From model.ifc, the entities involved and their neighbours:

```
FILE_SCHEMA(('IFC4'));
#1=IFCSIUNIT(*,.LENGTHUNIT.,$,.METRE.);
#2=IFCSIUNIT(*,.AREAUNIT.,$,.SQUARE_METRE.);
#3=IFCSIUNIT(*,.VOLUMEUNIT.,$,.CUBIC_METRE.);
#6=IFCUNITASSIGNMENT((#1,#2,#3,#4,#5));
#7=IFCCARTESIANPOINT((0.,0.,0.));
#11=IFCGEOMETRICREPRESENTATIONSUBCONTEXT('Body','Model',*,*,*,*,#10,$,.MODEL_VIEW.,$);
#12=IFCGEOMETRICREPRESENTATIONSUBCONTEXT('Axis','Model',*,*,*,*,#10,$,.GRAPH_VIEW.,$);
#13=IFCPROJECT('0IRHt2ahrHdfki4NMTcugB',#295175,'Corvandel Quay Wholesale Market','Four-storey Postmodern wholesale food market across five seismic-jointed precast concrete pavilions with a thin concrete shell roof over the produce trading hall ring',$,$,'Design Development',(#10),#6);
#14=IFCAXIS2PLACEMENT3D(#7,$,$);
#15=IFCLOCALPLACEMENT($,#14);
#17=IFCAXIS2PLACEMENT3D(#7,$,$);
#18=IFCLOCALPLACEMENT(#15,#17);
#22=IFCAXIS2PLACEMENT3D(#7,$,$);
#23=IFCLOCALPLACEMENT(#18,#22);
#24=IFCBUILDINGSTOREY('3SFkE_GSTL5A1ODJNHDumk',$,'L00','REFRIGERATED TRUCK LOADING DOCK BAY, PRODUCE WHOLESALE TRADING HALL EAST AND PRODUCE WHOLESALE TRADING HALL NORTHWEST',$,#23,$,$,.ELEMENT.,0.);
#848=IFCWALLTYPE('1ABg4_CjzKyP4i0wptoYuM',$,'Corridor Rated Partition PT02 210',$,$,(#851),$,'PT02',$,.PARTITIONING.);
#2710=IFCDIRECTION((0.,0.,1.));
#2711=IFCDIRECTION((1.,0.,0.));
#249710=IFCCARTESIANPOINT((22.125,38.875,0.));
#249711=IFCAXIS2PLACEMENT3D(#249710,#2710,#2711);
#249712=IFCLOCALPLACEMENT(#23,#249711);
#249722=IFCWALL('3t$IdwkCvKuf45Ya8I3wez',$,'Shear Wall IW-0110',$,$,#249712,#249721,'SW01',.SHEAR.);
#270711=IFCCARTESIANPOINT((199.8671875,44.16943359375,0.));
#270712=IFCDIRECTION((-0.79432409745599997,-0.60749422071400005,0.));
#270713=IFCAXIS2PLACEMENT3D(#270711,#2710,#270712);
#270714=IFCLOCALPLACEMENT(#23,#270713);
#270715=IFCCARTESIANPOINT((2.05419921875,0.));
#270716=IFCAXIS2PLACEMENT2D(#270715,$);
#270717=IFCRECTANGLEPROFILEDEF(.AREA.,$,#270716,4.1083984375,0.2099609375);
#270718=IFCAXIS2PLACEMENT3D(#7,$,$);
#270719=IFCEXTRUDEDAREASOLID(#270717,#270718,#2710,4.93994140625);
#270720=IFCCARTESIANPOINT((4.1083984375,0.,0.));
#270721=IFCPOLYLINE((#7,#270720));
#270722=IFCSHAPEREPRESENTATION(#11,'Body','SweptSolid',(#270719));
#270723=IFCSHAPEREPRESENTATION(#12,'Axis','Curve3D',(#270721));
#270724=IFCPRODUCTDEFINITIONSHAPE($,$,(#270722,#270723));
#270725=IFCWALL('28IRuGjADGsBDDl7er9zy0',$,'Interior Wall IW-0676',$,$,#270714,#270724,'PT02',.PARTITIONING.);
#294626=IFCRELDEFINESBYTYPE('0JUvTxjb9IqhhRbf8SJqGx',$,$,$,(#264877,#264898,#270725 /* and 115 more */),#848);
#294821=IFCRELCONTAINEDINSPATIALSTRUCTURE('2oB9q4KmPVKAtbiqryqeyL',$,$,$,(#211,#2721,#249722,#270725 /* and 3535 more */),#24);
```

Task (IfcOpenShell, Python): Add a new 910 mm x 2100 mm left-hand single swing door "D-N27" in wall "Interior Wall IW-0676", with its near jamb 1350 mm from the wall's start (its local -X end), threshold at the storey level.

```python
import numpy as np
import ifcopenshell
import ifcopenshell.api.feature
import ifcopenshell.api.geometry
import ifcopenshell.api.root
import ifcopenshell.api.spatial
import ifcopenshell.geom
import ifcopenshell.util.element
import ifcopenshell.util.placement
import ifcopenshell.util.representation
import ifcopenshell.util.shape
import ifcopenshell.util.unit

model = ifcopenshell.open("model.ifc")
unit_scale = ifcopenshell.util.unit.calculate_unit_scale(model)
settings = ifcopenshell.geom.settings()


def volume(element):
    """Net volume in cubic metres, openings subtracted."""
    shape = ifcopenshell.geom.create_shape(settings, element)
    return ifcopenshell.util.shape.get_volume(shape.geometry)


wall = model.by_guid("28IRuGjADGsBDDl7er9zy0")
storey = ifcopenshell.util.element.get_container(wall, ifc_class="IfcBuildingStorey")
context = ifcopenshell.util.representation.get_context(model, "Model", "Body", "MODEL_VIEW")
before = volume(wall)

width, height, from_end, sill = 0.91, 2.1, 1.35, 0.0  # metres

# The wall runs along its own X axis, and the end named is its -X end.
wall_shape = ifcopenshell.geom.create_shape(settings, wall)
x, y, z = ifcopenshell.util.shape.get_vertices(wall_shape.geometry).T
start = x.min() + from_end
face, thickness = float(y.min()), float(y.max() - y.min())
wall_matrix = ifcopenshell.util.placement.get_local_placement(wall.ObjectPlacement)
level = ifcopenshell.util.placement.get_local_placement(storey.ObjectPlacement)[2, 3]


def in_wall(x, y):
    """Placement at x, y metres in the wall's axes, at sill height."""
    matrix = wall_matrix.copy()
    matrix[:, 3] = wall_matrix @ np.array([x / unit_scale, y / unit_scale, 0.0, 1.0])
    matrix[2, 3] = level + sill / unit_scale
    return matrix


# Opening: a box that overshoots both wall faces by 50 mm.
opening = ifcopenshell.api.root.create_entity(model, ifc_class="IfcOpeningElement", predefined_type="OPENING")
box = ifcopenshell.api.geometry.add_wall_representation(
    model, context=context, length=width, height=height, thickness=thickness + 0.1
)
ifcopenshell.api.geometry.assign_representation(model, product=opening, representation=box)
ifcopenshell.api.geometry.edit_object_placement(model, product=opening, matrix=in_wall(start, face - 0.05), is_si=False)
ifcopenshell.api.feature.add_feature(model, feature=opening, element=wall)

door = ifcopenshell.api.root.create_entity(model, ifc_class="IfcDoor", name="D-N27", predefined_type="DOOR")
door.OverallWidth, door.OverallHeight = width / unit_scale, height / unit_scale
door.OperationType = "SINGLE_SWING_LEFT"
body = ifcopenshell.api.geometry.add_door_representation(
    model,
    context=context,
    overall_width=door.OverallWidth,
    overall_height=door.OverallHeight,
    operation_type="SINGLE_SWING_LEFT",
    lining_properties={"LiningDepth": thickness / unit_scale, "ThresholdDepth": thickness / unit_scale},
)
ifcopenshell.api.geometry.assign_representation(model, product=door, representation=body)
ifcopenshell.api.spatial.assign_container(model, products=[door], relating_structure=storey)
ifcopenshell.api.feature.add_filling(model, opening=opening, element=door)

# The lining spans the wall, so the door starts at the wall face.
ifcopenshell.api.geometry.edit_object_placement(model, product=door, matrix=in_wall(start, face), is_si=False)

after = volume(wall)

print(f"wall volume {before:.3f} -> {after:.3f} m3")

model.write("model_edited.ifc")
```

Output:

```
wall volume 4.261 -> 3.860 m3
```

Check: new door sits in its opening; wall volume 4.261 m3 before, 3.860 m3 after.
